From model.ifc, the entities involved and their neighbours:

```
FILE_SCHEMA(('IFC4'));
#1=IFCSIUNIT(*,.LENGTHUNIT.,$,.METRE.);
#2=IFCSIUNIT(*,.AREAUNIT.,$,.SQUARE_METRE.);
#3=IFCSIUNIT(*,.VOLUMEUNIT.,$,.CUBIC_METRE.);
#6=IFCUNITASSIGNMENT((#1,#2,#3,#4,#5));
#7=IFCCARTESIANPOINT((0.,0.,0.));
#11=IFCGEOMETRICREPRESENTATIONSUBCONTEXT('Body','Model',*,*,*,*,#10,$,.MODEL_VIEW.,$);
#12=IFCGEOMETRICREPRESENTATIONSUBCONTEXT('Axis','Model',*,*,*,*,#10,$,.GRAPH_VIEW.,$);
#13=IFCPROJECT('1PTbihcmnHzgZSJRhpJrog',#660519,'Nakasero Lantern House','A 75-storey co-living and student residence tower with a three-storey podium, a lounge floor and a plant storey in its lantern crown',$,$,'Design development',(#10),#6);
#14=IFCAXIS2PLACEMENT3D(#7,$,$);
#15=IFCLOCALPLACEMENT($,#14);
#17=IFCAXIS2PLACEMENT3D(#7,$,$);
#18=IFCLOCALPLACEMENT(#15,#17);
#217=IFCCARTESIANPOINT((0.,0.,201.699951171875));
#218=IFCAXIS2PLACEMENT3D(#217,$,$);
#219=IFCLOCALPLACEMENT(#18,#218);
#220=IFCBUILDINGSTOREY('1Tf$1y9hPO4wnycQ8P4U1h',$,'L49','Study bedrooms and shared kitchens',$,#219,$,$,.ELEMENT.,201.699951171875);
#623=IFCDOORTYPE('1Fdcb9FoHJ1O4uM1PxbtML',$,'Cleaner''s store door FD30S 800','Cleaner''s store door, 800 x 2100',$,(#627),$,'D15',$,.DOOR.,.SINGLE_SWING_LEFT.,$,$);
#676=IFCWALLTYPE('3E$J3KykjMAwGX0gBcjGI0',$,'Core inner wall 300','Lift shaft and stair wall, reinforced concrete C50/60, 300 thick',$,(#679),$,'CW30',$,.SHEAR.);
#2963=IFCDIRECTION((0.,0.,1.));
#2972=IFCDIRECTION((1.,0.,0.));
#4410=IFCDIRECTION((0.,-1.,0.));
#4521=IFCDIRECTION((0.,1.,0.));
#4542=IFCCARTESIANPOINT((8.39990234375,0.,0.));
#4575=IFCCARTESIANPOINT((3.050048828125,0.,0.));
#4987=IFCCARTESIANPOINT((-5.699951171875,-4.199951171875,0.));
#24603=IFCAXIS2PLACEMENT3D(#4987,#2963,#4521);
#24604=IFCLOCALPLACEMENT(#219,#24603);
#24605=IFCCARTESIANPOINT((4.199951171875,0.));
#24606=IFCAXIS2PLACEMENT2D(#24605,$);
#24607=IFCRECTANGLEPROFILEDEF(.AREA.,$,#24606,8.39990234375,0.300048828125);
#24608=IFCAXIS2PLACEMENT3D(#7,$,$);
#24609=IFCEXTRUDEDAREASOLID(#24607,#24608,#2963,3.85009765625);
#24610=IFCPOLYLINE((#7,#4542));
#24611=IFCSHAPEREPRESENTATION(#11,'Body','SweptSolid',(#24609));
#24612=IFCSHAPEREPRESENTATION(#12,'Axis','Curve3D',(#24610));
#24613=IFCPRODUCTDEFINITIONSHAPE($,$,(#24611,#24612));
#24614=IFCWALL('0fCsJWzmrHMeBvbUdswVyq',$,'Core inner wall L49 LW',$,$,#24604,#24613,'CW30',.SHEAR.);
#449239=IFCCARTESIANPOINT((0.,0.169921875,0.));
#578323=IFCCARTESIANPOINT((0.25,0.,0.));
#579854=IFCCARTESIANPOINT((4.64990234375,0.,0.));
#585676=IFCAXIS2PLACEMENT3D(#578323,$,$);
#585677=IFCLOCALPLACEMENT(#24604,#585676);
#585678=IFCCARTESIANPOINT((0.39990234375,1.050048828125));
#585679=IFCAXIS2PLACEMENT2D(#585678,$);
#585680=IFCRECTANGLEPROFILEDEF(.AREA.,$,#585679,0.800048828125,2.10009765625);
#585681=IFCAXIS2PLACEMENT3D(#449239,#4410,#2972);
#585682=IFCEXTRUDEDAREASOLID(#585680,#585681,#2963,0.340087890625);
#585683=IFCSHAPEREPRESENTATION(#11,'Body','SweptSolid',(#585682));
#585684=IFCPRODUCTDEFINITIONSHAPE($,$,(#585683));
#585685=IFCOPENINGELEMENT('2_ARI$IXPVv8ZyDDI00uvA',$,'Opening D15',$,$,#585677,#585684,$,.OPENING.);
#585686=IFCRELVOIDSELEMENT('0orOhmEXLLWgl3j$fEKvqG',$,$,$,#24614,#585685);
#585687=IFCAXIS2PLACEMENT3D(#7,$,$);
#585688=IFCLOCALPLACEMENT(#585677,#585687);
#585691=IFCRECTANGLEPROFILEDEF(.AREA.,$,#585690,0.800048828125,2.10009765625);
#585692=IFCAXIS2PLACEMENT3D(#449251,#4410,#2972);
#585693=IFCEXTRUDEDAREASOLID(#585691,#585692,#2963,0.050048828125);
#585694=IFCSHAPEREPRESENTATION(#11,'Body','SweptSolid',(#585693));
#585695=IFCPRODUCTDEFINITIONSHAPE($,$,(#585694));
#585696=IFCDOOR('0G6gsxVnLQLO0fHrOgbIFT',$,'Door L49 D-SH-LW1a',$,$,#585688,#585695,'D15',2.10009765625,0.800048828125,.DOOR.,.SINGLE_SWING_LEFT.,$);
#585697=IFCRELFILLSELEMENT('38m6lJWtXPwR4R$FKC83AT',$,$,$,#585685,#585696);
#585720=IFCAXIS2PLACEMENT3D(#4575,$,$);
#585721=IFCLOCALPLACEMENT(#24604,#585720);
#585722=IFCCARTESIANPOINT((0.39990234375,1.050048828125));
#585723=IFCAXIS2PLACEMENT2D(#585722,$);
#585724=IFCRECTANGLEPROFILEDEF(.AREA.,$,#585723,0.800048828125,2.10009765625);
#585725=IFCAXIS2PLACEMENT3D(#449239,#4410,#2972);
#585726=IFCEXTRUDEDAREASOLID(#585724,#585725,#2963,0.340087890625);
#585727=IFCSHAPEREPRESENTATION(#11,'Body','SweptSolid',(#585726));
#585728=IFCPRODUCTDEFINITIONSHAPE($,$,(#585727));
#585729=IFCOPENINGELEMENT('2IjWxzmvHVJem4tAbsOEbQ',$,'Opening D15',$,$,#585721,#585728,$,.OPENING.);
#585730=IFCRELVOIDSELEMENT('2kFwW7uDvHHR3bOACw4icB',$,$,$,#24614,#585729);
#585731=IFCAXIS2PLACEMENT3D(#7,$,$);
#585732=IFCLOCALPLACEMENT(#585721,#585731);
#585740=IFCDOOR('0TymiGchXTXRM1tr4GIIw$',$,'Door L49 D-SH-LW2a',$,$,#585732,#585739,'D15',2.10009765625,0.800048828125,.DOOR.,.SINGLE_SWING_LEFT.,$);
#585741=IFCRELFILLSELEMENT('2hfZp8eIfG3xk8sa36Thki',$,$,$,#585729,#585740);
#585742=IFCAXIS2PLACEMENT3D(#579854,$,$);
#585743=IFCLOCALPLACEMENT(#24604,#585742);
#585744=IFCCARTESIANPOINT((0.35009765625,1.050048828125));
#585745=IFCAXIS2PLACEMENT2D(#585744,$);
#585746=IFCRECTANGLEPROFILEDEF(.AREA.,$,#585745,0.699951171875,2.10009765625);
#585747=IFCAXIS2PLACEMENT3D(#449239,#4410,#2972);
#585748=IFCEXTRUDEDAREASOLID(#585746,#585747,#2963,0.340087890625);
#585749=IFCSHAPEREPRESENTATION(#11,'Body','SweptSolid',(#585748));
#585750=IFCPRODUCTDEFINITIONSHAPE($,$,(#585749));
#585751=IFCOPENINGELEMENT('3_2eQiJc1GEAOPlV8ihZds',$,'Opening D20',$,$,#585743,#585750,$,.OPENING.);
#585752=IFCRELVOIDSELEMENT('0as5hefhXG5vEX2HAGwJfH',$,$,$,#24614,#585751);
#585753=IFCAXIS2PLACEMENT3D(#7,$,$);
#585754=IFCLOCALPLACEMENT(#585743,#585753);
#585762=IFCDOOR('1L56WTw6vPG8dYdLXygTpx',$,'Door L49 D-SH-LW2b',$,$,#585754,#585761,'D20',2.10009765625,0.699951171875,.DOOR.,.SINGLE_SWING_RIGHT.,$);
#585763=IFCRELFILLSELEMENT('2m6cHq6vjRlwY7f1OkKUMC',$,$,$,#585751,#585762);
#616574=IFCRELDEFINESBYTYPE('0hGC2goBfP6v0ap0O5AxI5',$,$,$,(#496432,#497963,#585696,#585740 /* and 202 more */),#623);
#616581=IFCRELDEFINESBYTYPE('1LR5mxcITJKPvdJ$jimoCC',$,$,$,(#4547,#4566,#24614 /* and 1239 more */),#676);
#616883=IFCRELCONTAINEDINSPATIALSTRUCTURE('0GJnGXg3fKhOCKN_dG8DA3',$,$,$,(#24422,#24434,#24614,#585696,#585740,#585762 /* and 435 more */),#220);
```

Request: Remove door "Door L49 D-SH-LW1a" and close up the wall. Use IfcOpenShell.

```python
import ifcopenshell
import ifcopenshell.api.feature
import ifcopenshell.api.root
import ifcopenshell.geom
import ifcopenshell.util.shape

model = ifcopenshell.open("model.ifc")
settings = ifcopenshell.geom.settings()


def volume(element):
    """Net volume in cubic metres, openings subtracted."""
    shape = ifcopenshell.geom.create_shape(settings, element)
    return ifcopenshell.util.shape.get_volume(shape.geometry)


door = model.by_id(585696)
opening = door.FillsVoids[0].RelatingOpeningElement
wall = opening.VoidsElements[0].RelatingBuildingElement
before = volume(wall)

ifcopenshell.api.root.remove_product(model, product=door)
ifcopenshell.api.feature.remove_feature(model, feature=opening)

after = volume(wall)

print(f"wall volume {before:.3f} -> {after:.3f} m3")

model.write("model_v2.ifc")
```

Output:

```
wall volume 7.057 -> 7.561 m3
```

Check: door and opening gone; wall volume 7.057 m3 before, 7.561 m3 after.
